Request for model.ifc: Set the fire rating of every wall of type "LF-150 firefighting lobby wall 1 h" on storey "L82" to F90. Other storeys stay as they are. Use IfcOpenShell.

First a look at what the model holds.

```python
import ifcopenshell
import ifcopenshell.util.element

model = ifcopenshell.open("model.ifc")
print(model.schema)
storey = next(s for s in model.by_type("IfcBuildingStorey") if s.Name == "L82")
walls = [e for e in ifcopenshell.util.element.get_decomposition(storey) if e.is_a("IfcWall")]
seen = {}
for e in walls:
    element_type = ifcopenshell.util.element.get_type(e)
    key = (element_type.Name if element_type != e and element_type else None, ifcopenshell.util.element.get_pset(e, "Pset_WallCommon", "FireRating"))
    seen[key] = seen.get(key, 0) + 1
for (name, value), count in sorted(seen.items(), key=str):
    print(count, "x", name, "|", value)
```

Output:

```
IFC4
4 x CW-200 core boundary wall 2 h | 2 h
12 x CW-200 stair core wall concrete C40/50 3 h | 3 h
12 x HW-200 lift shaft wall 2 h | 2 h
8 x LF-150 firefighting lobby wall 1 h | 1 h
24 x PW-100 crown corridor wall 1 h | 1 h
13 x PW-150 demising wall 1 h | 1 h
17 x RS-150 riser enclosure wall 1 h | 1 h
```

```python
import ifcopenshell
import ifcopenshell.api.pset
import ifcopenshell.util.element

model = ifcopenshell.open("model.ifc")

storey = next(s for s in model.by_type("IfcBuildingStorey") if s.Name == "L82")
walls = [e for e in ifcopenshell.util.element.get_decomposition(storey) if e.is_a("IfcWall")]

count = 0
for e in walls:
    element_type = ifcopenshell.util.element.get_type(e)
    if element_type in (None, e) or element_type.Name != "LF-150 firefighting lobby wall 1 h":
        continue
    found = ifcopenshell.util.element.get_pset(e, "Pset_WallCommon", should_inherit=False)
    if found:
        pset = model.by_id(found["id"])
        if len(ifcopenshell.util.element.get_elements_by_pset(pset)) > 1:
            pset = ifcopenshell.api.pset.unshare_pset(model, products=[e], pset=pset)[0]
    else:
        pset = ifcopenshell.api.pset.add_pset(model, product=e, name="Pset_WallCommon")
    ifcopenshell.api.pset.edit_pset(model, pset=pset, properties={"FireRating": "F90"})
    count += 1

print(count, "walls updated")

model.write("model_v2.ifc")
```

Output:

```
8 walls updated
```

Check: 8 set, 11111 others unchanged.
